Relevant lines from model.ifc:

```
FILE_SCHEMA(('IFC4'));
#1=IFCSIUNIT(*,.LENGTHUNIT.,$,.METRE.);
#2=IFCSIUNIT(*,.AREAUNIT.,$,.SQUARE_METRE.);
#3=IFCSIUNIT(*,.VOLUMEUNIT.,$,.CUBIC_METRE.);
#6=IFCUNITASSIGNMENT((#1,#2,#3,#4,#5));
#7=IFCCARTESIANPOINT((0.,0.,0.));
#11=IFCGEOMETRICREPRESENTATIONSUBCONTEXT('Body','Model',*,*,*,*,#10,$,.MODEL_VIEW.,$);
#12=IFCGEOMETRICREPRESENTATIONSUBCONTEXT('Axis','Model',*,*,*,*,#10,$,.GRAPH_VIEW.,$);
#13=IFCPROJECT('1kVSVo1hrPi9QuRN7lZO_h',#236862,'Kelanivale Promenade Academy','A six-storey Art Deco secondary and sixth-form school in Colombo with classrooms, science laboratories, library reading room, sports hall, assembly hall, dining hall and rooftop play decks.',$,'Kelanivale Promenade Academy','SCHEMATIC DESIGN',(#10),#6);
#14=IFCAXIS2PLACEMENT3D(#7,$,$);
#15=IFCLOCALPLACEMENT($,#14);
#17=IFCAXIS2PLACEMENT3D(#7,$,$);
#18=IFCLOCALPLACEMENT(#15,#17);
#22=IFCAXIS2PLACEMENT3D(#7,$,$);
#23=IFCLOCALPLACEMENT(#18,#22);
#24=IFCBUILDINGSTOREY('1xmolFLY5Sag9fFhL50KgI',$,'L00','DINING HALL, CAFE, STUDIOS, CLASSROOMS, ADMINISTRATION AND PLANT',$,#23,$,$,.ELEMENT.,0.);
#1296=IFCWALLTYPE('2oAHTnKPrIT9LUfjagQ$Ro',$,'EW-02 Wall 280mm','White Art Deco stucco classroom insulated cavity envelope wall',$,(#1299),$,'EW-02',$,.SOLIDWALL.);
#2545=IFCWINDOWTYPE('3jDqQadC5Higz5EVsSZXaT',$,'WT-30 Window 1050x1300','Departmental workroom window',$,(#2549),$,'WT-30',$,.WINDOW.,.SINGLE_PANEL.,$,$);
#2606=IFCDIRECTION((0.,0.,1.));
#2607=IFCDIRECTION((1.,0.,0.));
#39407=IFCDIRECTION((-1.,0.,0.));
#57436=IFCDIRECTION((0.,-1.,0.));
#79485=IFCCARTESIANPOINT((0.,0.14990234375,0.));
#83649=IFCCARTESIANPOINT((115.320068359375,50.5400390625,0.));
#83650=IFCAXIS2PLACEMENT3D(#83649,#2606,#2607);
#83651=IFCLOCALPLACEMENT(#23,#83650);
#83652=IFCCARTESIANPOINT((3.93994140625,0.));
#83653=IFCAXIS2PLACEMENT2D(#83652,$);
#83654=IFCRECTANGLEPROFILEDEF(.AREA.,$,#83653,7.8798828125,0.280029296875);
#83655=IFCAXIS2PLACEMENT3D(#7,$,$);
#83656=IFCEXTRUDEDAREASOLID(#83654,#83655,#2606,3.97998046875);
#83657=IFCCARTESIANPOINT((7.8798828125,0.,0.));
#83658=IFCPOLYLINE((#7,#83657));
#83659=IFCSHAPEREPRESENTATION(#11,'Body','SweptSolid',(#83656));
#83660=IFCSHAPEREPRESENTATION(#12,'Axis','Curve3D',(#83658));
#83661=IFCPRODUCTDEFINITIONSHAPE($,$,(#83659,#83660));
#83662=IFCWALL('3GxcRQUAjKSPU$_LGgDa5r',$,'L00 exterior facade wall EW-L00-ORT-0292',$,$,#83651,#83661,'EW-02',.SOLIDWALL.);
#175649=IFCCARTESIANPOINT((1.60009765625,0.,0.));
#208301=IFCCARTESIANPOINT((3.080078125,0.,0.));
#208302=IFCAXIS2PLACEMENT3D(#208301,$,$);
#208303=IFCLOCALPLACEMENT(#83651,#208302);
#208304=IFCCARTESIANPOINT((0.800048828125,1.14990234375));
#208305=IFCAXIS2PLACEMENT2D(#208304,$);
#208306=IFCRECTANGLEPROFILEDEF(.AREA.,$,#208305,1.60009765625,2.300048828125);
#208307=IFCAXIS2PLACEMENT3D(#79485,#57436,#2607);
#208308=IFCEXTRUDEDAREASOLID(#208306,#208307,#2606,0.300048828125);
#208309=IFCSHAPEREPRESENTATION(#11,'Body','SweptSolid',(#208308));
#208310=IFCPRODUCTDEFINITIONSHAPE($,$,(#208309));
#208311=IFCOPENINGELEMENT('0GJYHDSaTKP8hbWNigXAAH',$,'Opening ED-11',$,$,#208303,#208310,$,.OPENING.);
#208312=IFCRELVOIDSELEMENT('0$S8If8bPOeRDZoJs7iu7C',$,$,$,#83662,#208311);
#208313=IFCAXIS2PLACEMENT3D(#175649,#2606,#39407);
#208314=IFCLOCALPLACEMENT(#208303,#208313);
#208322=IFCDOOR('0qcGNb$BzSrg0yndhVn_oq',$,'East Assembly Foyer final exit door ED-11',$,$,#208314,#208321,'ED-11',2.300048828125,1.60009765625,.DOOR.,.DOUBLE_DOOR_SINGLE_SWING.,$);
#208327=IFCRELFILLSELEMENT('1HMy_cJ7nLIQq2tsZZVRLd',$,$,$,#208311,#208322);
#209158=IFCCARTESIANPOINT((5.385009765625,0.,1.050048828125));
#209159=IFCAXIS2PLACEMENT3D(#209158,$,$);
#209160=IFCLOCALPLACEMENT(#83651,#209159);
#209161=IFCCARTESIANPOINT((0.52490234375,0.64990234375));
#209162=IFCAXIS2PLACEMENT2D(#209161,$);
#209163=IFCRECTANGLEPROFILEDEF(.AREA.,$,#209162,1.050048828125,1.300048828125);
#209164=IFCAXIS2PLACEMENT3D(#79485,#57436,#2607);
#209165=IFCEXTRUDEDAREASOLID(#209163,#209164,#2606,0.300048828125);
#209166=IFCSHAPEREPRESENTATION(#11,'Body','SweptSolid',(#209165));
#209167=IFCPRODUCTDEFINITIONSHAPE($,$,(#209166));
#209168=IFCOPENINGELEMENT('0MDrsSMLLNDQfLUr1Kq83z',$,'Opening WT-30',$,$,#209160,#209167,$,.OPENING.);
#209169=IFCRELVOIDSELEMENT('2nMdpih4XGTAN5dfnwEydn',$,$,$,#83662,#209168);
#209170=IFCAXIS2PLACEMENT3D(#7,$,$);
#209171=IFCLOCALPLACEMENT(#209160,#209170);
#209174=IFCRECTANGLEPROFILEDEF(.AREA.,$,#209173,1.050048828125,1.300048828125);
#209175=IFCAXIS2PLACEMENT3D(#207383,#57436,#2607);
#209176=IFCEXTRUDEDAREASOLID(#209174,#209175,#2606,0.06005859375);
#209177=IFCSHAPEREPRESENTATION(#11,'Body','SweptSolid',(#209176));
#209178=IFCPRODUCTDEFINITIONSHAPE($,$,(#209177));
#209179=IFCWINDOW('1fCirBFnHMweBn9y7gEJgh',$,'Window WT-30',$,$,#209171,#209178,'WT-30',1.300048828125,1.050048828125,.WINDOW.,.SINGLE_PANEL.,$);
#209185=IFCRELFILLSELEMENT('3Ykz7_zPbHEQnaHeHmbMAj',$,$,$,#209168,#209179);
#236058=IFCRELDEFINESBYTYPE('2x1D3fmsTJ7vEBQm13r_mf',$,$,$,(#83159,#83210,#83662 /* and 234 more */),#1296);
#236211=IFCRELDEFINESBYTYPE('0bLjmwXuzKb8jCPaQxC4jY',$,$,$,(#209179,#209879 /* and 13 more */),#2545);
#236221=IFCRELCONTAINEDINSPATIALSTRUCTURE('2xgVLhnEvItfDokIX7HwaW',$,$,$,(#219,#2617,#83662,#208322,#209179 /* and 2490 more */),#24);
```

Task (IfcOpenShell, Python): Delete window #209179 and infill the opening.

```python
import ifcopenshell
import ifcopenshell.api.feature
import ifcopenshell.api.root
import ifcopenshell.geom
import ifcopenshell.util.shape

model = ifcopenshell.open("model.ifc")
settings = ifcopenshell.geom.settings()


def volume(element):
    """Net volume in cubic metres, openings subtracted."""
    shape = ifcopenshell.geom.create_shape(settings, element)
    return ifcopenshell.util.shape.get_volume(shape.geometry)


window = model.by_guid("1fCirBFnHMweBn9y7gEJgh")
opening = window.FillsVoids[0].RelatingOpeningElement
wall = opening.VoidsElements[0].RelatingBuildingElement
before = volume(wall)

ifcopenshell.api.root.remove_product(model, product=window)
ifcopenshell.api.feature.remove_feature(model, feature=opening)

after = volume(wall)

print(f"wall volume {before:.3f} -> {after:.3f} m3")

model.write("model_edited.ifc")
```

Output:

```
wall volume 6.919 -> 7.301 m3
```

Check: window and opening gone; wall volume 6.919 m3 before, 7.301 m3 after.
